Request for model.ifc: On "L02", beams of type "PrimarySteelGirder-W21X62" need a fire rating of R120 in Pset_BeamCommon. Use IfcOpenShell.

First a look at what the model holds.

```python
import ifcopenshell
import ifcopenshell.util.element

model = ifcopenshell.open("model.ifc")
print(model.schema)
storey = next(s for s in model.by_type("IfcBuildingStorey") if s.Name == "L02")
beams = [e for e in ifcopenshell.util.element.get_decomposition(storey) if e.is_a("IfcBeam")]
seen = {}
for e in beams:
    element_type = ifcopenshell.util.element.get_type(e)
    key = (element_type.Name if element_type != e and element_type else None, ifcopenshell.util.element.get_pset(e, "Pset_BeamCommon", "FireRating"))
    seen[key] = seen.get(key, 0) + 1
for (name, value), count in sorted(seen.items(), key=str):
    print(count, "x", name, "|", value)
```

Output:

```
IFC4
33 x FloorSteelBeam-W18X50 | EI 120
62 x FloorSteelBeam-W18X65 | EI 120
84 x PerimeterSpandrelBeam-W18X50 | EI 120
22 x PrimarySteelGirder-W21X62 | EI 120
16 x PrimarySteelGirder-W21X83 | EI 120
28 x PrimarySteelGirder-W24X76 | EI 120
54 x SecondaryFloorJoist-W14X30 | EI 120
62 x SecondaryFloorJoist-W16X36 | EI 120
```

```python
import ifcopenshell
import ifcopenshell.api.pset
import ifcopenshell.util.element

model = ifcopenshell.open("model.ifc")

storey = next(s for s in model.by_type("IfcBuildingStorey") if s.Name == "L02")
beams = [e for e in ifcopenshell.util.element.get_decomposition(storey) if e.is_a("IfcBeam")]

count = 0
for e in beams:
    element_type = ifcopenshell.util.element.get_type(e)
    if element_type in (None, e) or element_type.Name != "PrimarySteelGirder-W21X62":
        continue
    # add_pset returns the element's existing set when there is one.
    pset = ifcopenshell.api.pset.add_pset(model, product=e, name="Pset_BeamCommon")
    ifcopenshell.api.pset.edit_pset(model, pset=pset, properties={"FireRating": "R120"})
    count += 1

print(count, "beams updated")

model.write("model_v2.ifc")
```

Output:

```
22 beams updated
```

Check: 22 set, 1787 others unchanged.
